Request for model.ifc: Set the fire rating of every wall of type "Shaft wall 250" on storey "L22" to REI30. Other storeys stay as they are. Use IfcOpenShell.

First a look at what the model holds.

```python
import ifcopenshell
import ifcopenshell.util.element

model = ifcopenshell.open("model.ifc")
print(model.schema)
storey = next(s for s in model.by_type("IfcBuildingStorey") if s.Name == "L22")
walls = [e for e in ifcopenshell.util.element.get_decomposition(storey) if e.is_a("IfcWall")]
seen = {}
for e in walls:
    element_type = ifcopenshell.util.element.get_type(e)
    key = (element_type.Name if element_type != e and element_type else None, ifcopenshell.util.element.get_pset(e, "Pset_WallCommon", "FireRating"))
    seen[key] = seen.get(key, 0) + 1
for (name, value), count in sorted(seen.items(), key=str):
    print(count, "x", name, "|", value)
```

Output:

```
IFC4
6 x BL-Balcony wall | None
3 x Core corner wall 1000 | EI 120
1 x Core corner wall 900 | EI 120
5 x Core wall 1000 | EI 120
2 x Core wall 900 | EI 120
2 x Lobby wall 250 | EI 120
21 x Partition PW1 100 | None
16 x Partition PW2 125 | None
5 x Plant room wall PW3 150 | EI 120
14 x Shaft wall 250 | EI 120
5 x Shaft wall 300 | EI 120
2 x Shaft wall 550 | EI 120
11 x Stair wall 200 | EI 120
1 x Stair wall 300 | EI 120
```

```python
import ifcopenshell
import ifcopenshell.api.pset
import ifcopenshell.util.element

model = ifcopenshell.open("model.ifc")

storey = next(s for s in model.by_type("IfcBuildingStorey") if s.Name == "L22")
walls = [e for e in ifcopenshell.util.element.get_decomposition(storey) if e.is_a("IfcWall")]

count = 0
for e in walls:
    element_type = ifcopenshell.util.element.get_type(e)
    if element_type in (None, e) or element_type.Name != "Shaft wall 250":
        continue
    found = ifcopenshell.util.element.get_pset(e, "Pset_WallCommon", should_inherit=False)
    if found:
        pset = model.by_id(found["id"])
        if len(ifcopenshell.util.element.get_elements_by_pset(pset)) > 1:
            pset = ifcopenshell.api.pset.unshare_pset(model, products=[e], pset=pset)[0]
    else:
        pset = ifcopenshell.api.pset.add_pset(model, product=e, name="Pset_WallCommon")
    ifcopenshell.api.pset.edit_pset(model, pset=pset, properties={"FireRating": "REI30"})
    count += 1

print(count, "walls updated")

model.write("model-out.ifc")
```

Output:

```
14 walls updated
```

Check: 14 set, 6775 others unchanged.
